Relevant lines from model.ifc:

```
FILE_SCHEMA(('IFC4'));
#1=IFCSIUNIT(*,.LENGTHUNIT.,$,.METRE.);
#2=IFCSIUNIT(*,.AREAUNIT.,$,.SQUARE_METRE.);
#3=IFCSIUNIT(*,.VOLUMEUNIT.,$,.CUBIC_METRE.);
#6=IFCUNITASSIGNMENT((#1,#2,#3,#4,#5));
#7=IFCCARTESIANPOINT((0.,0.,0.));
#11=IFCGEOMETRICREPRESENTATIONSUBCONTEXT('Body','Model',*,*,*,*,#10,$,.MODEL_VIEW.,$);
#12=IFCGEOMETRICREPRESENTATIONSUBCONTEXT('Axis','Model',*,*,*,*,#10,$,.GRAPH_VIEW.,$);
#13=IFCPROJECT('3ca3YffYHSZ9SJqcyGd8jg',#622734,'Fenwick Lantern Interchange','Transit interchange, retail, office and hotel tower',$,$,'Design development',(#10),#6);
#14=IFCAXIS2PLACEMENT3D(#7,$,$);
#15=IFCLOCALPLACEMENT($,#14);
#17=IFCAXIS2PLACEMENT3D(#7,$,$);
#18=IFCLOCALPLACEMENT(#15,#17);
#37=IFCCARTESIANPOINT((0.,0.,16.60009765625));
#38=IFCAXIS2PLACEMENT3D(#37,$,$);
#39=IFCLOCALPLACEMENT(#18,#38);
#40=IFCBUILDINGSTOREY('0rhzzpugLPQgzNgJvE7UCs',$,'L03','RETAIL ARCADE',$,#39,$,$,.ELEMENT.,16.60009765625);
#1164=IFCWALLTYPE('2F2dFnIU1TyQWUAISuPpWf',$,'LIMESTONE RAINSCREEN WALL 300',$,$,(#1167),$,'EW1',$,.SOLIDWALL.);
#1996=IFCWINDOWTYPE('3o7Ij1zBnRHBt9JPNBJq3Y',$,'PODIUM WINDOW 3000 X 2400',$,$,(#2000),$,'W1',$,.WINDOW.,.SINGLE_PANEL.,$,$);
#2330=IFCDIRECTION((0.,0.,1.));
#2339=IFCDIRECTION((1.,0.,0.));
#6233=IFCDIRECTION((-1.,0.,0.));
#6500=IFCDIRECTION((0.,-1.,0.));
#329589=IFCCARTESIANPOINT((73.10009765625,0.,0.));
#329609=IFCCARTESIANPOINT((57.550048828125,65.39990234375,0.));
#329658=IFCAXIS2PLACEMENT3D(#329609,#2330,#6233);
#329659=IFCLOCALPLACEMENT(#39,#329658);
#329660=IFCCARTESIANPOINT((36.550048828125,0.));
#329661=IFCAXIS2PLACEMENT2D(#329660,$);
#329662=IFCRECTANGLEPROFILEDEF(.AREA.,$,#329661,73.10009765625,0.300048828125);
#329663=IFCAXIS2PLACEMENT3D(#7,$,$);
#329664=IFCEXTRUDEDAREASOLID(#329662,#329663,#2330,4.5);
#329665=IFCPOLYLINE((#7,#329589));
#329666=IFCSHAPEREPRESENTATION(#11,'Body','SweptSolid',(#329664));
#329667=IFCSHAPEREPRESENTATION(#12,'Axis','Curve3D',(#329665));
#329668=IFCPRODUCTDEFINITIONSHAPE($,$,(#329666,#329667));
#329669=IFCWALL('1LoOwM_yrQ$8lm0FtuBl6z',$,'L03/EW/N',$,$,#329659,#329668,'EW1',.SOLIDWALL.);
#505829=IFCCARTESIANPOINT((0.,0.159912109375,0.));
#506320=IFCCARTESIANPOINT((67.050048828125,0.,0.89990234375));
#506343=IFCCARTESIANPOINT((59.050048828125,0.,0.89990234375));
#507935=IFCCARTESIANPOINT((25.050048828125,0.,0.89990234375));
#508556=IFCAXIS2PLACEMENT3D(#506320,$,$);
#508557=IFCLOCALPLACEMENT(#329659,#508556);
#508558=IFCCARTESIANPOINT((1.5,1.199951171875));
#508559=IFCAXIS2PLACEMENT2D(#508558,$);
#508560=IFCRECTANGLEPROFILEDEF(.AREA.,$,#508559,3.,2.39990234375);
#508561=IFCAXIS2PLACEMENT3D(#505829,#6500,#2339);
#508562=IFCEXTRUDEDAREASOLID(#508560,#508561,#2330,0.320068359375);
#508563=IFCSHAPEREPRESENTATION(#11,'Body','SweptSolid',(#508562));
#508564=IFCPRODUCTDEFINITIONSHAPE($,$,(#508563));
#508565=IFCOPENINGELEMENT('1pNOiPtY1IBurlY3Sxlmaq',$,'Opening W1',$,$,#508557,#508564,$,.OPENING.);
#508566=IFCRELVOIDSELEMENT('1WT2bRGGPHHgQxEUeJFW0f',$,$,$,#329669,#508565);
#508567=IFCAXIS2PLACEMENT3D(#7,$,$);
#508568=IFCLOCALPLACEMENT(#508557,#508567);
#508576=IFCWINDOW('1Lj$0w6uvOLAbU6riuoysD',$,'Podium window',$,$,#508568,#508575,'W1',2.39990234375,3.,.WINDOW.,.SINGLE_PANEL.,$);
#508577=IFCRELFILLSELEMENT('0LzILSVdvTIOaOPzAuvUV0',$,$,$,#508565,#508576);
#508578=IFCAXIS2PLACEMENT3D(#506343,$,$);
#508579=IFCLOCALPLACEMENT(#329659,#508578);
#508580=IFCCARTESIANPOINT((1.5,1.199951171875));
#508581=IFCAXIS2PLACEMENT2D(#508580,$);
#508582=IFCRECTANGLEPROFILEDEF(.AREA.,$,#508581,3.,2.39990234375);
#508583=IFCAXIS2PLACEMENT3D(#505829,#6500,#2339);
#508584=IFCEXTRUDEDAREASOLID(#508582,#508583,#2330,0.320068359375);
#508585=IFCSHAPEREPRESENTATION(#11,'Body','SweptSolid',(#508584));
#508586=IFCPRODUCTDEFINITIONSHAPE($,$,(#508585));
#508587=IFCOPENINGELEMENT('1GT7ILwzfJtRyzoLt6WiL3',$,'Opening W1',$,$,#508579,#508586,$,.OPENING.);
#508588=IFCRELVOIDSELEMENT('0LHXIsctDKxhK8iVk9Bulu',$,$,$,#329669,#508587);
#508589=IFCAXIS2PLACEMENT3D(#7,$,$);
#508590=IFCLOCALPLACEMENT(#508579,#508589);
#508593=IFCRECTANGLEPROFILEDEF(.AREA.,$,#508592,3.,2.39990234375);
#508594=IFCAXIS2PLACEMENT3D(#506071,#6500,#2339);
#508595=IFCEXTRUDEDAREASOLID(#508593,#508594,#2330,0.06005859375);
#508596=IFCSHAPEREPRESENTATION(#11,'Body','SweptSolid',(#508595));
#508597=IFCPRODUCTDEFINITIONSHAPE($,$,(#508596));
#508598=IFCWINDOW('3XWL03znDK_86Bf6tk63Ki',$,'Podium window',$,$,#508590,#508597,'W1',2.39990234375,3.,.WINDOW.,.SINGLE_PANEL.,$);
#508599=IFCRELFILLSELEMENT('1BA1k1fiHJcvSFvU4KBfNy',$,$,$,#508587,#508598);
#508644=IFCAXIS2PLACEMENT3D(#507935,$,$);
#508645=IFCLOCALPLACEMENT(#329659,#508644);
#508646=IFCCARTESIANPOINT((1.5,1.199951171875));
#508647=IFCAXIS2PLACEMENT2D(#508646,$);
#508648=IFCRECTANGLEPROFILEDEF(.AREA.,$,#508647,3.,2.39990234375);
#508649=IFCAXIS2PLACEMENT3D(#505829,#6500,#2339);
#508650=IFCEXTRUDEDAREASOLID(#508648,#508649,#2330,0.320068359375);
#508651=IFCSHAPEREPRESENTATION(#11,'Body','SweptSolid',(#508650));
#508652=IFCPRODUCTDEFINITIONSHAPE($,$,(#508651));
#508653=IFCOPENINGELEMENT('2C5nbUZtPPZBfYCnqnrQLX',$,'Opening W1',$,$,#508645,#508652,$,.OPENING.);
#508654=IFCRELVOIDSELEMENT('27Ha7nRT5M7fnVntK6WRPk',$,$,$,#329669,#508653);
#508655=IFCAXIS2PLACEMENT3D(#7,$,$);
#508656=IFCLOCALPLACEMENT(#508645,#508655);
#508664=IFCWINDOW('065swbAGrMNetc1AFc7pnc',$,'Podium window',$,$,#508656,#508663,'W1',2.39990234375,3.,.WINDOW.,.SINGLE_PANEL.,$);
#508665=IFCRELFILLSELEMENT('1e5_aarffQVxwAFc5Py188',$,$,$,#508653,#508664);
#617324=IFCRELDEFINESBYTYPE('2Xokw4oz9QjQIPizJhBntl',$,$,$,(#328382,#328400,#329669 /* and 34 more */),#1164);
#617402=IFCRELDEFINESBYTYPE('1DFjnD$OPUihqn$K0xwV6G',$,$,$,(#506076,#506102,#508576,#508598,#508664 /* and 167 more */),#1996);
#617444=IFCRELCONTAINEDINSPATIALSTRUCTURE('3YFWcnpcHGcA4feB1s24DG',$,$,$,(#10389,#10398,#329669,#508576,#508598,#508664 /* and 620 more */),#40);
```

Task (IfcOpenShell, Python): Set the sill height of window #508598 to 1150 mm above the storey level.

```python
import numpy as np
import ifcopenshell
import ifcopenshell.api.geometry
import ifcopenshell.geom
import ifcopenshell.util.element
import ifcopenshell.util.placement
import ifcopenshell.util.shape
import ifcopenshell.util.unit

model = ifcopenshell.open("model.ifc")
unit_scale = ifcopenshell.util.unit.calculate_unit_scale(model)

window = model.by_guid("3XWL03znDK_86Bf6tk63Ki")
opening = window.FillsVoids[0].RelatingOpeningElement
storey = ifcopenshell.util.element.get_container(window, ifc_class="IfcBuildingStorey")
level = ifcopenshell.util.placement.get_local_placement(storey.ObjectPlacement)[2, 3]

# The opening's origin need not be at the sill, so measure its lowest point.
shape = ifcopenshell.geom.create_shape(ifcopenshell.geom.settings(), opening)
bottom = ifcopenshell.util.shape.get_shape_bottom_elevation(shape, shape.geometry) / unit_scale
dz = level + 1.15 / unit_scale - bottom

shift = np.array([0.0, 0.0, dz])
# The window is placed relative to its opening, so it follows when the opening moves.
matrix = ifcopenshell.util.placement.get_local_placement(opening.ObjectPlacement)
matrix[:3, 3] += shift
ifcopenshell.api.geometry.edit_object_placement(
    model, product=opening, matrix=matrix, is_si=False, should_transform_children=True
)

print(f"moved by {dz * unit_scale:+.3f} m")

model.write("model_edited.ifc")
```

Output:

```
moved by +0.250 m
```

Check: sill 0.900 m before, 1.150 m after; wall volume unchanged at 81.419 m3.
